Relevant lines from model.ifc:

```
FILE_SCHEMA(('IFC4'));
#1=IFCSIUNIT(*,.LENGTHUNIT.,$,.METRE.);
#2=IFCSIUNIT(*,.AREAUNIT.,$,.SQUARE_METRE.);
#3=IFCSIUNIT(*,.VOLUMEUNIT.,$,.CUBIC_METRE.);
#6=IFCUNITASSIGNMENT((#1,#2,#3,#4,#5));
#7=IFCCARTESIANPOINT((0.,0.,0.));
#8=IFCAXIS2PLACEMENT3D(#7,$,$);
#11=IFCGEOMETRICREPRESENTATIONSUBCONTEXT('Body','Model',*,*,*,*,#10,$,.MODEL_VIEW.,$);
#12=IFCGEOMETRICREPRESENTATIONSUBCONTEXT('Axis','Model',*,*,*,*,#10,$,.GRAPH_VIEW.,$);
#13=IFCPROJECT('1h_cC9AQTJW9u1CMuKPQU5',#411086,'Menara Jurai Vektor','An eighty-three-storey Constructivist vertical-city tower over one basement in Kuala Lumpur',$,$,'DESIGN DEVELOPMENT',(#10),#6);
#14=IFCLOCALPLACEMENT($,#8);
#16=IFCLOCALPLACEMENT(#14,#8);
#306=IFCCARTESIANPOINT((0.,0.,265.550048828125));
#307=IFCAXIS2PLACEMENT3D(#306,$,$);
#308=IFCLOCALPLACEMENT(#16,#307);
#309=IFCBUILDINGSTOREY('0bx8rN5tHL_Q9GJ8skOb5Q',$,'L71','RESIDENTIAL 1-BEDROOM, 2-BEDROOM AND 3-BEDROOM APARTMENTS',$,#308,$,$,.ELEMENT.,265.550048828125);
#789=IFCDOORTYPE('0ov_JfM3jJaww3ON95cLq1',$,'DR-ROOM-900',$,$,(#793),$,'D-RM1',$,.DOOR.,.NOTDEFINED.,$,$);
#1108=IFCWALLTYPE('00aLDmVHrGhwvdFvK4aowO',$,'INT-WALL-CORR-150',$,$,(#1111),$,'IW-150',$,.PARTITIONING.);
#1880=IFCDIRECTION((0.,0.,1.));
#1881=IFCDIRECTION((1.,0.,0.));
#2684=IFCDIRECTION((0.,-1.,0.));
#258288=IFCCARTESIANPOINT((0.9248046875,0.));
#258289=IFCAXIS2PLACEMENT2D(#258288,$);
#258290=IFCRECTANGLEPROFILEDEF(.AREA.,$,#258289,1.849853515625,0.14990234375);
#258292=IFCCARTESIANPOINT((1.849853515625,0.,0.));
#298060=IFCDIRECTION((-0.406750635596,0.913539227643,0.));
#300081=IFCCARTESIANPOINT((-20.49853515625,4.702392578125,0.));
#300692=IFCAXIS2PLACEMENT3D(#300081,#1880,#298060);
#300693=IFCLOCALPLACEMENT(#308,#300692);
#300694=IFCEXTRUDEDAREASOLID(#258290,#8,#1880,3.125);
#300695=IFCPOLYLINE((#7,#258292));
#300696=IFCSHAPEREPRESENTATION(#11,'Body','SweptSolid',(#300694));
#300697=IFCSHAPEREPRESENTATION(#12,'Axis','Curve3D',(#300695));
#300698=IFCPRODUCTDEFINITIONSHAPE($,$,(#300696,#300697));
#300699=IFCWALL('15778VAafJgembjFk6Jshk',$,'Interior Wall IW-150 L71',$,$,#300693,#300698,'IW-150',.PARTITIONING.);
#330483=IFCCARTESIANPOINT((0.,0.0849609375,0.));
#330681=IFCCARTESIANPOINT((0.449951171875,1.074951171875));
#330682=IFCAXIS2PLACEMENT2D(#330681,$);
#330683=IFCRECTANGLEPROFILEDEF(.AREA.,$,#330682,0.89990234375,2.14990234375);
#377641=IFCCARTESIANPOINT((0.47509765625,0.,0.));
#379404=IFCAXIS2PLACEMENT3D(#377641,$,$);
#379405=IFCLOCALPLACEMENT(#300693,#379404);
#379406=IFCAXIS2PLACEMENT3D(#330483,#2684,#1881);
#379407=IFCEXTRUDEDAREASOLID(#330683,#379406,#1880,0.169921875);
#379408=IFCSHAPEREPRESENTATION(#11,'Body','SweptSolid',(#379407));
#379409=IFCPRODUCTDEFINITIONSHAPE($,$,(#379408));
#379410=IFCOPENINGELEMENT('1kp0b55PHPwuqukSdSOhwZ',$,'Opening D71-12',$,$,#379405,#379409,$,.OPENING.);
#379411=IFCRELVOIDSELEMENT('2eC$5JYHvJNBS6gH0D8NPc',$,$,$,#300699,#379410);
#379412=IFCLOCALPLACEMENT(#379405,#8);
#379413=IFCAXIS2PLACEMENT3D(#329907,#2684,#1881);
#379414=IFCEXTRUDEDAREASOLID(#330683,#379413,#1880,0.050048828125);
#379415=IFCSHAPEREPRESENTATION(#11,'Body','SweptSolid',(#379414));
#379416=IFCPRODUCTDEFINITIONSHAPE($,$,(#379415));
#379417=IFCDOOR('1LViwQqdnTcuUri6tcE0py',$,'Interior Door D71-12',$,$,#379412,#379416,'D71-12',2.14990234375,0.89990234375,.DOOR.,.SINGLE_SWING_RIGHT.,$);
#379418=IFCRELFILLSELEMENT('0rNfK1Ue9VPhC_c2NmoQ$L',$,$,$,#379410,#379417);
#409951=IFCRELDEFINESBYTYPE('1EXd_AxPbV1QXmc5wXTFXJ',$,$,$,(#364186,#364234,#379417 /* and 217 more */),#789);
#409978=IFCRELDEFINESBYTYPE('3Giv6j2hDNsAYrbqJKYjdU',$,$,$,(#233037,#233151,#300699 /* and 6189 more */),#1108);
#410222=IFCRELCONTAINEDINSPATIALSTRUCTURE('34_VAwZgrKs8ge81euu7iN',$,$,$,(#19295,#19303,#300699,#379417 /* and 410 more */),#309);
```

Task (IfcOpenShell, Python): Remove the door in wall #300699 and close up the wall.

```python
import ifcopenshell
import ifcopenshell.api.feature
import ifcopenshell.api.root
import ifcopenshell.geom
import ifcopenshell.util.shape

model = ifcopenshell.open("model.ifc")
settings = ifcopenshell.geom.settings()


def volume(element):
    """Net volume in cubic metres, openings subtracted."""
    shape = ifcopenshell.geom.create_shape(settings, element)
    return ifcopenshell.util.shape.get_volume(shape.geometry)


door = model.by_id(379417)
opening = door.FillsVoids[0].RelatingOpeningElement
wall = opening.VoidsElements[0].RelatingBuildingElement
before = volume(wall)

ifcopenshell.api.root.remove_product(model, product=door)
ifcopenshell.api.feature.remove_feature(model, feature=opening)

after = volume(wall)

print(f"wall volume {before:.3f} -> {after:.3f} m3")

model.write("model_edited.ifc")
```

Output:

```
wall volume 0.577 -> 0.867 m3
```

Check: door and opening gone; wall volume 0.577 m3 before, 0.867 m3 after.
